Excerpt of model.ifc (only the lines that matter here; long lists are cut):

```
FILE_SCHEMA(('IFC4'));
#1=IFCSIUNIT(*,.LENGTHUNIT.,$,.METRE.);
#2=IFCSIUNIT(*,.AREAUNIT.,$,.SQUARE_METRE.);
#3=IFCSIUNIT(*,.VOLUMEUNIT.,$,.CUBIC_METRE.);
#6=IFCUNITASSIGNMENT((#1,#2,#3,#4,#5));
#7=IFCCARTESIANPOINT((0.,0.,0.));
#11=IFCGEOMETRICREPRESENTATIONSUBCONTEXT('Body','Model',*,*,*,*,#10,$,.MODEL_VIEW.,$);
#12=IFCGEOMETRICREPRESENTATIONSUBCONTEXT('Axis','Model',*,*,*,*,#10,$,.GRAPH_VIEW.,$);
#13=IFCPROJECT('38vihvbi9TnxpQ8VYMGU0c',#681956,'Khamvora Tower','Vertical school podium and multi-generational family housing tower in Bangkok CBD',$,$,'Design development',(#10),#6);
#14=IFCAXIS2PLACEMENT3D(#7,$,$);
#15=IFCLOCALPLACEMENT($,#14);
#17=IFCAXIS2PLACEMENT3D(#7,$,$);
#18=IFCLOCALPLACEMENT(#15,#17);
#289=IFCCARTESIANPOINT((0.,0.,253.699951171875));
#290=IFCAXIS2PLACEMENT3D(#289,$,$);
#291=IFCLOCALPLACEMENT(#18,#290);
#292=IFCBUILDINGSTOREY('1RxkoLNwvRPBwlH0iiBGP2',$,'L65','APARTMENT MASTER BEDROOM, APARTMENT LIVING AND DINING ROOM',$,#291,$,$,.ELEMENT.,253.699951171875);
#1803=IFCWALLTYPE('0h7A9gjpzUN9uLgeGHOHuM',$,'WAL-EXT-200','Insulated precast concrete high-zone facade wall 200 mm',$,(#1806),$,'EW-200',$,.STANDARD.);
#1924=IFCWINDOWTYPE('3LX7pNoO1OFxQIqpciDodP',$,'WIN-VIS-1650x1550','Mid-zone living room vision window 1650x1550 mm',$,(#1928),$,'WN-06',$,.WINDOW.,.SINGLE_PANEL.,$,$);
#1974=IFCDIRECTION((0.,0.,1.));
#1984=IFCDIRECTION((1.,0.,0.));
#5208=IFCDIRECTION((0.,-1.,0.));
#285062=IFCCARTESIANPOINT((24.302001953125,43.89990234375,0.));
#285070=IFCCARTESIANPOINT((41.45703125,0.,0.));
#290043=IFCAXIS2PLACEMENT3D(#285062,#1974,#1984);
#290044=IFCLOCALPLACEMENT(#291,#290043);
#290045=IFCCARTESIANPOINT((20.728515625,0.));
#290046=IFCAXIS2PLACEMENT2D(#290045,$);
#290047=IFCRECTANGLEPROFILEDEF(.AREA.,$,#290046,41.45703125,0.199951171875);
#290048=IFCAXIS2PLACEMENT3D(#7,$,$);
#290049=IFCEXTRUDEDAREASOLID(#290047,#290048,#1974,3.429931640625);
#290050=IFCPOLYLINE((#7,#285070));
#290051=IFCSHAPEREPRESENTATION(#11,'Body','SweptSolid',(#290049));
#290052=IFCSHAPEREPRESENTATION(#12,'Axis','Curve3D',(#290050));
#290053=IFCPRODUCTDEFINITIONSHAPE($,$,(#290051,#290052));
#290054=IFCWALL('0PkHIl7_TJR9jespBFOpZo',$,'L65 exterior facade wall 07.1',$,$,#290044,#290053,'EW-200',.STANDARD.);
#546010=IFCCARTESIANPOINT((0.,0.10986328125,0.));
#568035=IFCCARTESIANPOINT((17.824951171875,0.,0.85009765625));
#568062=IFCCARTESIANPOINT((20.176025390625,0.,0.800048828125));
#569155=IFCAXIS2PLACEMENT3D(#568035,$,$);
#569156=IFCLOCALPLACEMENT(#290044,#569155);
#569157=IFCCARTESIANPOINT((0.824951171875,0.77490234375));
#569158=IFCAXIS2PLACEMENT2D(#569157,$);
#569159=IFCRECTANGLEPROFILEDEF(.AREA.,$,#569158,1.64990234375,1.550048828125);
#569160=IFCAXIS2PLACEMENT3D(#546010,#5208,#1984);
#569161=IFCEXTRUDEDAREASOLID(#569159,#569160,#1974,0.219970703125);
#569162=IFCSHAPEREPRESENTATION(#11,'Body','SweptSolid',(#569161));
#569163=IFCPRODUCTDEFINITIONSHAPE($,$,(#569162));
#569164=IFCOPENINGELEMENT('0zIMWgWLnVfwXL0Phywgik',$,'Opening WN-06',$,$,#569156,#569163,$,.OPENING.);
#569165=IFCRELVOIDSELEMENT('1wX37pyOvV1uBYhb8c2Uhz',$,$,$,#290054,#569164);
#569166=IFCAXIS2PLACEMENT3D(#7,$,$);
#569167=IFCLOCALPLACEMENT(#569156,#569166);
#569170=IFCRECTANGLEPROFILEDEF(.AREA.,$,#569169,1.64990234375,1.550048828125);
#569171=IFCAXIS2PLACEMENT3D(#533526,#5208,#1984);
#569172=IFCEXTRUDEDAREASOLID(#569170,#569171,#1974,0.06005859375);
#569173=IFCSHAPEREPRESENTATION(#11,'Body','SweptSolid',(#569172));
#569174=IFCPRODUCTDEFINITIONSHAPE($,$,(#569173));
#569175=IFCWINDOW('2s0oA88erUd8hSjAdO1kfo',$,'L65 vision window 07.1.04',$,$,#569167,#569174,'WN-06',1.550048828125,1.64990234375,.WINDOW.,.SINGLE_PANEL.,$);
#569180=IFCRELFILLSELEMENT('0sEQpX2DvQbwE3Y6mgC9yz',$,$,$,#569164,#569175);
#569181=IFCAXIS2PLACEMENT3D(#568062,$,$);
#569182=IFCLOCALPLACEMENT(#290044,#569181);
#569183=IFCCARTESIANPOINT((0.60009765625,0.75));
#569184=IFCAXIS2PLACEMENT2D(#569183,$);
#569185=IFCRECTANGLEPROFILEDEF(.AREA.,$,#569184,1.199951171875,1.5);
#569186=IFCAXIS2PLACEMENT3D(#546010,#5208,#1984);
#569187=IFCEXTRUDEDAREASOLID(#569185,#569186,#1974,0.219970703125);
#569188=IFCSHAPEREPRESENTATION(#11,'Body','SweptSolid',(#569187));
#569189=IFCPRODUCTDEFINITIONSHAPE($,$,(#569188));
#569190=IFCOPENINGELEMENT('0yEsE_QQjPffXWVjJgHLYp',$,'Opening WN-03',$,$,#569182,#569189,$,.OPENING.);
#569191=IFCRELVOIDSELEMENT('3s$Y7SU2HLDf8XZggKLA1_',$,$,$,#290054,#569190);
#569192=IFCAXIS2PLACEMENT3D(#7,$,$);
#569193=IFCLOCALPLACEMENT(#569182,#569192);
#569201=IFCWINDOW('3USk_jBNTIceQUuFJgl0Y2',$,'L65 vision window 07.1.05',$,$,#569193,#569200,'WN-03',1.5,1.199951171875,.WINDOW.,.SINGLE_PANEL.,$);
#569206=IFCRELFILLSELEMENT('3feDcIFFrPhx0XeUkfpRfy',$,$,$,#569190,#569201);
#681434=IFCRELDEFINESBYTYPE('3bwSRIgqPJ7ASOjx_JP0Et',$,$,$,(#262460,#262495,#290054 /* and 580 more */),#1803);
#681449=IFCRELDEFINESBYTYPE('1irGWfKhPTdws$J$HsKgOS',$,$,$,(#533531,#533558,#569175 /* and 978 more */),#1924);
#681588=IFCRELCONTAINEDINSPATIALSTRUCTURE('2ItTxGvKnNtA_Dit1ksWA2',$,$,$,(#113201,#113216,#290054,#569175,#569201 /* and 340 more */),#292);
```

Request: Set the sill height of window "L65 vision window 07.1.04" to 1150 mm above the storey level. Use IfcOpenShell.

```python
import numpy as np
import ifcopenshell
import ifcopenshell.api.geometry
import ifcopenshell.geom
import ifcopenshell.util.element
import ifcopenshell.util.placement
import ifcopenshell.util.shape
import ifcopenshell.util.unit

model = ifcopenshell.open("model.ifc")
unit_scale = ifcopenshell.util.unit.calculate_unit_scale(model)

window = model.by_guid("2s0oA88erUd8hSjAdO1kfo")
opening = window.FillsVoids[0].RelatingOpeningElement
storey = ifcopenshell.util.element.get_container(window, ifc_class="IfcBuildingStorey")
level = ifcopenshell.util.placement.get_local_placement(storey.ObjectPlacement)[2, 3]

# The opening's origin need not be at the sill, so measure its lowest point.
shape = ifcopenshell.geom.create_shape(ifcopenshell.geom.settings(), opening)
bottom = ifcopenshell.util.shape.get_shape_bottom_elevation(shape, shape.geometry) / unit_scale
dz = level + 1.15 / unit_scale - bottom

shift = np.array([0.0, 0.0, dz])
# The window is placed relative to its opening, so it follows when the opening moves.
matrix = ifcopenshell.util.placement.get_local_placement(opening.ObjectPlacement)
matrix[:3, 3] += shift
ifcopenshell.api.geometry.edit_object_placement(
    model, product=opening, matrix=matrix, is_si=False, should_transform_children=True
)

print(f"moved by {dz * unit_scale:+.3f} m")

model.write("model_rev.ifc")
```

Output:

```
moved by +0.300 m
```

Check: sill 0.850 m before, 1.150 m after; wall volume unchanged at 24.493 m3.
